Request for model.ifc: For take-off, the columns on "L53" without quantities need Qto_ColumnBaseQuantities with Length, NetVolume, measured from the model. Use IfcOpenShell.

First a look at what the model holds.

```python
import ifcopenshell
import ifcopenshell.util.element
import ifcopenshell.util.unit

model = ifcopenshell.open("model.ifc")
print(model.schema)
for unit_type in ("LENGTHUNIT", "AREAUNIT", "VOLUMEUNIT"):
    print(unit_type, ifcopenshell.util.unit.calculate_unit_scale(model, unit_type))
storey = next(s for s in model.by_type("IfcBuildingStorey") if s.Name == "L53")
columns = [e for e in ifcopenshell.util.element.get_decomposition(storey) if e.is_a("IfcColumn")]
for e in sorted(columns, key=lambda e: e.id()):
    print(e.id(), e.is_a(), e.Name, list(ifcopenshell.util.element.get_psets(e, qtos_only=True)), sep=" | ")
```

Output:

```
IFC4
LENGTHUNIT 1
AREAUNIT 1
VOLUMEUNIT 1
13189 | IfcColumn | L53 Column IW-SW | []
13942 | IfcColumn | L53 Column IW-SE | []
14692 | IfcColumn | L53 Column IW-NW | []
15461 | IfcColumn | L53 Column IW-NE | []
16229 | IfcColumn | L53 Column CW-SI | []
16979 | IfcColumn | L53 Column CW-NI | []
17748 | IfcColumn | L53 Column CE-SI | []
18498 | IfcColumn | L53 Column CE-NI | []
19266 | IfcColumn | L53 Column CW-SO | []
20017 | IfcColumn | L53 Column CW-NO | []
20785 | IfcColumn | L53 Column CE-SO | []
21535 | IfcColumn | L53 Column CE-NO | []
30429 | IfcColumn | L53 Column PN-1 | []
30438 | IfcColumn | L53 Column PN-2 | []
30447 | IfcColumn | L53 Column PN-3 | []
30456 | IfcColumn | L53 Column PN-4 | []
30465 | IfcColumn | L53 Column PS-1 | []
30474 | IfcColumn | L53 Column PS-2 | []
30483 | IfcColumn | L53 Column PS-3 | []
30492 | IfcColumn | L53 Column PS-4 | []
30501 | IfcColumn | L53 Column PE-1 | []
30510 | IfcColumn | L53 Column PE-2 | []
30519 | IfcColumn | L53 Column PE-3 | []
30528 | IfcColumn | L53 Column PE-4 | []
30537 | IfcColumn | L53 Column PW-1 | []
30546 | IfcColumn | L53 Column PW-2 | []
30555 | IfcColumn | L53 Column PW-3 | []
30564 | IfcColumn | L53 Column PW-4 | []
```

```python
import ifcopenshell
import ifcopenshell.api.pset
import ifcopenshell.geom
import ifcopenshell.util.element
import ifcopenshell.util.shape
import ifcopenshell.util.unit

model = ifcopenshell.open("model.ifc")
unit_scale = ifcopenshell.util.unit.calculate_unit_scale(model)
volume_scale = ifcopenshell.util.unit.calculate_unit_scale(model, "VOLUMEUNIT")
settings = ifcopenshell.geom.settings()

storey = next(s for s in model.by_type("IfcBuildingStorey") if s.Name == "L53")
columns = [e for e in ifcopenshell.util.element.get_decomposition(storey) if e.is_a("IfcColumn")]

for e in sorted(columns, key=lambda e: e.id()):
    if ifcopenshell.util.element.get_psets(e, qtos_only=True, should_inherit=False):
        continue
    # Geometry comes back in metres, in the element's own axes.
    shape = ifcopenshell.geom.create_shape(settings, e)
    values = {
        "Length": ifcopenshell.util.shape.get_z(shape.geometry) / unit_scale,
        "NetVolume": ifcopenshell.util.shape.get_volume(shape.geometry) / volume_scale,
    }
    qto = ifcopenshell.api.pset.add_qto(model, product=e, name="Qto_ColumnBaseQuantities")
    ifcopenshell.api.pset.edit_qto(model, qto=qto, properties=values)
    print(e.id(), {k: round(v, 3) for k, v in values.items()})

model.write("model-out.ifc")
```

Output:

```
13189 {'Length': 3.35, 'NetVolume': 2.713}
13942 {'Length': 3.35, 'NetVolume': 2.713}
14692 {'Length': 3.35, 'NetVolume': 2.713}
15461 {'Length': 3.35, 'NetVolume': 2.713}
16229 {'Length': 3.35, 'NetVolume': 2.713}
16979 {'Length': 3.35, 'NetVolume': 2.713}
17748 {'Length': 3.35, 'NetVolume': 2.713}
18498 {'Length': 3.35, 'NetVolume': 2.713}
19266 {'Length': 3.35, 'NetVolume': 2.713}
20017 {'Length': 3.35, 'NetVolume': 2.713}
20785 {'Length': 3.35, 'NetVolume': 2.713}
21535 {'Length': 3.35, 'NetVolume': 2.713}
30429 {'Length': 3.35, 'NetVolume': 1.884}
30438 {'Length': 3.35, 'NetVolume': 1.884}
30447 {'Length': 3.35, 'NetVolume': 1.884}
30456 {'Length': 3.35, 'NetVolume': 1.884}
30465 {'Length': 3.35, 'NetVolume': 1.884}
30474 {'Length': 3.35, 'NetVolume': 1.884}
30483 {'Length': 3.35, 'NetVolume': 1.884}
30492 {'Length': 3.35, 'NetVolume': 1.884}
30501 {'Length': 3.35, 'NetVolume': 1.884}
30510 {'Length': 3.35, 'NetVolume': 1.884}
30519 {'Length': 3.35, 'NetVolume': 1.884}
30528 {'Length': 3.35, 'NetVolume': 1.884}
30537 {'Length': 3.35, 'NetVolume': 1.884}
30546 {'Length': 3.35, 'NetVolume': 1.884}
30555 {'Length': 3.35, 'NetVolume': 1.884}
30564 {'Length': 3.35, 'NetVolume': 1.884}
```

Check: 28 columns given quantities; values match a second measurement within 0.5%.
